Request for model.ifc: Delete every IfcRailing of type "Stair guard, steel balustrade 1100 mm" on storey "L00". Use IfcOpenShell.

First a look at what the model holds.

```python
import ifcopenshell
import ifcopenshell.util.element

model = ifcopenshell.open("model.ifc")
print(model.schema)
storey = next(s for s in model.by_type("IfcBuildingStorey") if s.Name == "L00")
railings = [e for e in ifcopenshell.util.element.get_decomposition(storey) if e.is_a("IfcRailing")]
seen = {}
for e in railings:
    element_type = ifcopenshell.util.element.get_type(e)
    name = element_type.Name if element_type not in (None, e) else None
    seen[name] = seen.get(name, 0) + 1
for name, count in sorted(seen.items(), key=str):
    print(count, "x", name)
```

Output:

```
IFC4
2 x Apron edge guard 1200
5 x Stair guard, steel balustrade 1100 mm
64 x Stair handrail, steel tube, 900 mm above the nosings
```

```python
import ifcopenshell
import ifcopenshell.api.root
import ifcopenshell.util.element

model = ifcopenshell.open("model.ifc")

storey = next(s for s in model.by_type("IfcBuildingStorey") if s.Name == "L00")
railings = [e for e in ifcopenshell.util.element.get_decomposition(storey) if e.is_a("IfcRailing")]
targets = [e for e in railings if (t := ifcopenshell.util.element.get_type(e)) not in (None, e) and t.Name == "Stair guard, steel balustrade 1100 mm"]

for e in targets:
    ifcopenshell.api.root.remove_product(model, product=e)
print(len(targets), "removed")

model.write("model_updated.ifc")
```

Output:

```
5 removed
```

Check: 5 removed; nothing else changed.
